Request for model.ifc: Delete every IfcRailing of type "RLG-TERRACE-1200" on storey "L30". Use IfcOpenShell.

First a look at what the model holds.

```python
import ifcopenshell
import ifcopenshell.util.element

model = ifcopenshell.open("model.ifc")
print(model.schema)
storey = next(s for s in model.by_type("IfcBuildingStorey") if s.Name == "L30")
railings = [e for e in ifcopenshell.util.element.get_decomposition(storey) if e.is_a("IfcRailing")]
seen = {}
for e in railings:
    element_type = ifcopenshell.util.element.get_type(e)
    name = element_type.Name if element_type not in (None, e) else None
    seen[name] = seen.get(name, 0) + 1
for name, count in sorted(seen.items(), key=str):
    print(count, "x", name)
```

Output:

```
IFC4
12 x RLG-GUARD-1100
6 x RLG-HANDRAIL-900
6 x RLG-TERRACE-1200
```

```python
import ifcopenshell
import ifcopenshell.api.root
import ifcopenshell.util.element

model = ifcopenshell.open("model.ifc")

storey = next(s for s in model.by_type("IfcBuildingStorey") if s.Name == "L30")
railings = [e for e in ifcopenshell.util.element.get_decomposition(storey) if e.is_a("IfcRailing")]
targets = [e for e in railings if (t := ifcopenshell.util.element.get_type(e)) not in (None, e) and t.Name == "RLG-TERRACE-1200"]

for e in targets:
    ifcopenshell.api.root.remove_product(model, product=e)
print(len(targets), "removed")

model.write("model_updated.ifc")
```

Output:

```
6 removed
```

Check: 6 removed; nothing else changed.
